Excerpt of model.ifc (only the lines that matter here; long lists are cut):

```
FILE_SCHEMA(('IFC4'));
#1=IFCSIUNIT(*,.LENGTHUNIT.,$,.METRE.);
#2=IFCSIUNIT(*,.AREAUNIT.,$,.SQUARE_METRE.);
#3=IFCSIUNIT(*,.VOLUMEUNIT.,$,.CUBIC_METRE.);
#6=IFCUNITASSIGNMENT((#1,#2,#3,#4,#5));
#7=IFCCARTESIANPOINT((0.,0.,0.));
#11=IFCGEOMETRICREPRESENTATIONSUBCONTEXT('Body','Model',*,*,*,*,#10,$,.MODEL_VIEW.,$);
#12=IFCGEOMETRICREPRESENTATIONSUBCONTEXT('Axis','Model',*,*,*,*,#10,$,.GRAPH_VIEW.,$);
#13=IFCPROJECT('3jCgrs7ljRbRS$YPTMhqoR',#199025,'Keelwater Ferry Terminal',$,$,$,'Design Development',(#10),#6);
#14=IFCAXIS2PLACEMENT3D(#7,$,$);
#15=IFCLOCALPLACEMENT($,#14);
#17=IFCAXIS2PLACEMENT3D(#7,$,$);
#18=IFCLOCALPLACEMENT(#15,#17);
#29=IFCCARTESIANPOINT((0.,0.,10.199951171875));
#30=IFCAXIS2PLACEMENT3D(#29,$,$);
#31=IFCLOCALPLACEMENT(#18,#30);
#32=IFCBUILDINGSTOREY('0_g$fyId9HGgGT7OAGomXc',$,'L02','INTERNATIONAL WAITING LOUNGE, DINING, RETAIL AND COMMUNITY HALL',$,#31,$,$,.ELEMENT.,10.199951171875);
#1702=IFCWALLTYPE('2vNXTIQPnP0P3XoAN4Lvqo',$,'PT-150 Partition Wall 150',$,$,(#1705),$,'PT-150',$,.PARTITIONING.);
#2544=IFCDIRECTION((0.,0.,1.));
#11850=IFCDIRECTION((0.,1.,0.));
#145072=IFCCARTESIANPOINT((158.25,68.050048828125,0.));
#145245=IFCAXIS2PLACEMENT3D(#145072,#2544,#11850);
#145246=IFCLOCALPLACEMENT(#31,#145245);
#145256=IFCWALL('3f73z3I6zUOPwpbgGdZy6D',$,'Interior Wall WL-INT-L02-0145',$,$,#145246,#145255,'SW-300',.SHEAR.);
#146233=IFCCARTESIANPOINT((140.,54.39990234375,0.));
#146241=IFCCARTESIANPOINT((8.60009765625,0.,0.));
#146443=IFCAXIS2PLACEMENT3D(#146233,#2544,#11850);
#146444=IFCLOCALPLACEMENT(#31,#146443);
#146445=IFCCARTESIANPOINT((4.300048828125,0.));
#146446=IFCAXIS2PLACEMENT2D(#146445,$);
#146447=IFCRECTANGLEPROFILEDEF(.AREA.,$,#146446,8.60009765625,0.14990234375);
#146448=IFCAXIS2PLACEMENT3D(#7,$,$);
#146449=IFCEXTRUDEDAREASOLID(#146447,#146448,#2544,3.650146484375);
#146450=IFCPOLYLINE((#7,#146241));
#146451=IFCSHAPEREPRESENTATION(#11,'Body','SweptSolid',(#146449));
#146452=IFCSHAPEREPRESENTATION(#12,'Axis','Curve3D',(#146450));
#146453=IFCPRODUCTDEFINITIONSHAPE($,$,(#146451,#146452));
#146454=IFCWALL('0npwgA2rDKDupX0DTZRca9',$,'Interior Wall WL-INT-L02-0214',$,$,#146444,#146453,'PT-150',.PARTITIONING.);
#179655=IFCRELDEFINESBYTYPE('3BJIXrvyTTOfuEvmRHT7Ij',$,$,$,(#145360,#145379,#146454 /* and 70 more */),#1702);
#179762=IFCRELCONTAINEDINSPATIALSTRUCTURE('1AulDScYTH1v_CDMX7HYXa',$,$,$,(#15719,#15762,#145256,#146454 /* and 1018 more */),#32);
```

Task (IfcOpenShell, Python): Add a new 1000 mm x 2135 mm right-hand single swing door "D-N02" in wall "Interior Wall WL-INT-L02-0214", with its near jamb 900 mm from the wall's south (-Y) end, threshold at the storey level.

```python
import numpy as np
import ifcopenshell
import ifcopenshell.api.feature
import ifcopenshell.api.geometry
import ifcopenshell.api.root
import ifcopenshell.api.spatial
import ifcopenshell.geom
import ifcopenshell.util.element
import ifcopenshell.util.placement
import ifcopenshell.util.representation
import ifcopenshell.util.shape
import ifcopenshell.util.unit

model = ifcopenshell.open("model.ifc")
unit_scale = ifcopenshell.util.unit.calculate_unit_scale(model)
settings = ifcopenshell.geom.settings()


def volume(element):
    """Net volume in cubic metres, openings subtracted."""
    shape = ifcopenshell.geom.create_shape(settings, element)
    return ifcopenshell.util.shape.get_volume(shape.geometry)


wall = model.by_guid("0npwgA2rDKDupX0DTZRca9")
storey = ifcopenshell.util.element.get_container(wall, ifc_class="IfcBuildingStorey")
context = ifcopenshell.util.representation.get_context(model, "Model", "Body", "MODEL_VIEW")
before = volume(wall)

width, height, from_end, sill = 1, 2.135, 0.9, 0.0  # metres

# The wall runs along its own X axis, and the end named is its -X end.
wall_shape = ifcopenshell.geom.create_shape(settings, wall)
x, y, z = ifcopenshell.util.shape.get_vertices(wall_shape.geometry).T
start = x.min() + from_end
face, thickness = float(y.min()), float(y.max() - y.min())
wall_matrix = ifcopenshell.util.placement.get_local_placement(wall.ObjectPlacement)
level = ifcopenshell.util.placement.get_local_placement(storey.ObjectPlacement)[2, 3]


def in_wall(x, y):
    """Placement at x, y metres in the wall's axes, at sill height."""
    matrix = wall_matrix.copy()
    matrix[:, 3] = wall_matrix @ np.array([x / unit_scale, y / unit_scale, 0.0, 1.0])
    matrix[2, 3] = level + sill / unit_scale
    return matrix


# Opening: a box that overshoots both wall faces by 50 mm.
opening = ifcopenshell.api.root.create_entity(model, ifc_class="IfcOpeningElement", predefined_type="OPENING")
box = ifcopenshell.api.geometry.add_wall_representation(
    model, context=context, length=width, height=height, thickness=thickness + 0.1
)
ifcopenshell.api.geometry.assign_representation(model, product=opening, representation=box)
ifcopenshell.api.geometry.edit_object_placement(model, product=opening, matrix=in_wall(start, face - 0.05), is_si=False)
ifcopenshell.api.feature.add_feature(model, feature=opening, element=wall)

door = ifcopenshell.api.root.create_entity(model, ifc_class="IfcDoor", name="D-N02", predefined_type="DOOR")
door.OverallWidth, door.OverallHeight = width / unit_scale, height / unit_scale
door.OperationType = "SINGLE_SWING_RIGHT"
body = ifcopenshell.api.geometry.add_door_representation(
    model,
    context=context,
    overall_width=door.OverallWidth,
    overall_height=door.OverallHeight,
    operation_type="SINGLE_SWING_RIGHT",
    lining_properties={"LiningDepth": thickness / unit_scale, "ThresholdDepth": thickness / unit_scale},
)
ifcopenshell.api.geometry.assign_representation(model, product=door, representation=body)
ifcopenshell.api.spatial.assign_container(model, products=[door], relating_structure=storey)
ifcopenshell.api.feature.add_filling(model, opening=opening, element=door)

# The lining spans the wall, so the door starts at the wall face.
ifcopenshell.api.geometry.edit_object_placement(model, product=door, matrix=in_wall(start, face), is_si=False)

after = volume(wall)

print(f"wall volume {before:.3f} -> {after:.3f} m3")

model.write("model_edited.ifc")
```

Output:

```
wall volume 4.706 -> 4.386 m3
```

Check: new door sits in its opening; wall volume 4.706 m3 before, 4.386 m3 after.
